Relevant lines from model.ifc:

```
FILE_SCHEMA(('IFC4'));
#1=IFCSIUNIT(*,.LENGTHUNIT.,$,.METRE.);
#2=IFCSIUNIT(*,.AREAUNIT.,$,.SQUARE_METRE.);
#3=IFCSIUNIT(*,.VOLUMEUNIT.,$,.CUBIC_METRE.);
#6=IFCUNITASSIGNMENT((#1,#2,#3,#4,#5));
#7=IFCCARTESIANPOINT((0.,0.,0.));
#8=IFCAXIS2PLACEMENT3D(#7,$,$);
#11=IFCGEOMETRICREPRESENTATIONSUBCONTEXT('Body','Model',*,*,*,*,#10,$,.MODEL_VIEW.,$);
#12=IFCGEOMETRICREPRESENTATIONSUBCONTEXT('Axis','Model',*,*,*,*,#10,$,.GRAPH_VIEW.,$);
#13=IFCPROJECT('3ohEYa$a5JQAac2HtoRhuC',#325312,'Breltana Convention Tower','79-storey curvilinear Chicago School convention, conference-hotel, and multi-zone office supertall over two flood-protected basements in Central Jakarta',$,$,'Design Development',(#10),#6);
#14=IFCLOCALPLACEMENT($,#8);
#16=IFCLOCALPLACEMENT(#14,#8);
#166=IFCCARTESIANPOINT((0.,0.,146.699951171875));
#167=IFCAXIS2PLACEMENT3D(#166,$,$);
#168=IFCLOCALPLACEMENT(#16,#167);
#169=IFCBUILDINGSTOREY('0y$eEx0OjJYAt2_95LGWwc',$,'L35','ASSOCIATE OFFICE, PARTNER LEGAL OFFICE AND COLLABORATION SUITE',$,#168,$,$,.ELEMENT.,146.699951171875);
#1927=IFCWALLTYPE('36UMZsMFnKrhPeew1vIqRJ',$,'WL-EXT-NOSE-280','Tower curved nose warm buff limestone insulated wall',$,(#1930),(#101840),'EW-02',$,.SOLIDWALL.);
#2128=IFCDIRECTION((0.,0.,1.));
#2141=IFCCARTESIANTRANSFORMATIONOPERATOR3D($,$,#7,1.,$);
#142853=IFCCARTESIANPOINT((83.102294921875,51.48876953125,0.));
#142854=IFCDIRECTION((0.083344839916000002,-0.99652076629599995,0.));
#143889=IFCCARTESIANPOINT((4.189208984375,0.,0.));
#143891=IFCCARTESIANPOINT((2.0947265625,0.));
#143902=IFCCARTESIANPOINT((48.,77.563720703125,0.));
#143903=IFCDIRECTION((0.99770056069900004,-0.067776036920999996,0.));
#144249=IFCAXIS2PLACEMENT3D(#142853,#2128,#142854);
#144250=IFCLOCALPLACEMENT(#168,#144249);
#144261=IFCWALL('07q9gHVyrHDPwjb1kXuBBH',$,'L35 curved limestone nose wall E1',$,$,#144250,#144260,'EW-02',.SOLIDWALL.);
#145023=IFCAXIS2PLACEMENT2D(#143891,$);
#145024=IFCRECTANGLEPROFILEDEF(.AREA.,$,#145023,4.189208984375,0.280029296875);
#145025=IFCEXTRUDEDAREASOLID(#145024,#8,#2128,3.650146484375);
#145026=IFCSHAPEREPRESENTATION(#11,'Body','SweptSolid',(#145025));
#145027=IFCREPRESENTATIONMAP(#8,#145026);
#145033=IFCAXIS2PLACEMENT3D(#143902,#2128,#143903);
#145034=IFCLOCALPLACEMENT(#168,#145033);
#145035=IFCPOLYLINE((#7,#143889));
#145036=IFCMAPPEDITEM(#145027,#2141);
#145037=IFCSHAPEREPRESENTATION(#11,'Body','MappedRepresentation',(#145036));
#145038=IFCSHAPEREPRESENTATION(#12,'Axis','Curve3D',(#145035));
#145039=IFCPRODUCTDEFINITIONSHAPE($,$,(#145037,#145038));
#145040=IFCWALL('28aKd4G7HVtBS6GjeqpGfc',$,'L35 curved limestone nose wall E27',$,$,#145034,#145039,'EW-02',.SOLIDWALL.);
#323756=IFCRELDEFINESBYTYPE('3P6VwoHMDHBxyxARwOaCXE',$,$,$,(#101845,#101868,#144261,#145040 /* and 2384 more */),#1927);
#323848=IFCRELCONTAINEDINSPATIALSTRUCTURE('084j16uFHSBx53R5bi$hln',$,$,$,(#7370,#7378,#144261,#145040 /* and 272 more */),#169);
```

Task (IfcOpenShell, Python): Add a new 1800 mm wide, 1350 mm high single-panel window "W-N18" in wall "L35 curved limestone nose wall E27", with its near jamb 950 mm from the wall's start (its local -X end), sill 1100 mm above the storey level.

```python
import numpy as np
import ifcopenshell
import ifcopenshell.api.feature
import ifcopenshell.api.geometry
import ifcopenshell.api.root
import ifcopenshell.api.spatial
import ifcopenshell.geom
import ifcopenshell.util.element
import ifcopenshell.util.placement
import ifcopenshell.util.representation
import ifcopenshell.util.shape
import ifcopenshell.util.unit

model = ifcopenshell.open("model.ifc")
unit_scale = ifcopenshell.util.unit.calculate_unit_scale(model)
settings = ifcopenshell.geom.settings()


def volume(element):
    """Net volume in cubic metres, openings subtracted."""
    shape = ifcopenshell.geom.create_shape(settings, element)
    return ifcopenshell.util.shape.get_volume(shape.geometry)


wall = model.by_id(145040)
storey = ifcopenshell.util.element.get_container(wall, ifc_class="IfcBuildingStorey")
context = ifcopenshell.util.representation.get_context(model, "Model", "Body", "MODEL_VIEW")
before = volume(wall)

width, height, from_end, sill = 1.8, 1.35, 0.95, 1.1  # metres

# The wall runs along its own X axis, and the end named is its -X end.
wall_shape = ifcopenshell.geom.create_shape(settings, wall)
x, y, z = ifcopenshell.util.shape.get_vertices(wall_shape.geometry).T
start = x.min() + from_end
face, thickness = float(y.min()), float(y.max() - y.min())
wall_matrix = ifcopenshell.util.placement.get_local_placement(wall.ObjectPlacement)
level = ifcopenshell.util.placement.get_local_placement(storey.ObjectPlacement)[2, 3]


def in_wall(x, y):
    """Placement at x, y metres in the wall's axes, at sill height."""
    matrix = wall_matrix.copy()
    matrix[:, 3] = wall_matrix @ np.array([x / unit_scale, y / unit_scale, 0.0, 1.0])
    matrix[2, 3] = level + sill / unit_scale
    return matrix


# Opening: a box that overshoots both wall faces by 50 mm.
opening = ifcopenshell.api.root.create_entity(model, ifc_class="IfcOpeningElement", predefined_type="OPENING")
box = ifcopenshell.api.geometry.add_wall_representation(
    model, context=context, length=width, height=height, thickness=thickness + 0.1
)
ifcopenshell.api.geometry.assign_representation(model, product=opening, representation=box)
ifcopenshell.api.geometry.edit_object_placement(model, product=opening, matrix=in_wall(start, face - 0.05), is_si=False)
ifcopenshell.api.feature.add_feature(model, feature=opening, element=wall)

window = ifcopenshell.api.root.create_entity(model, ifc_class="IfcWindow", name="W-N18", predefined_type="WINDOW")
window.OverallWidth, window.OverallHeight = width / unit_scale, height / unit_scale
window.PartitioningType = "SINGLE_PANEL"
body = ifcopenshell.api.geometry.add_window_representation(
    model,
    context=context,
    overall_width=window.OverallWidth,
    overall_height=window.OverallHeight,
    partition_type="SINGLE_PANEL",
)
ifcopenshell.api.geometry.assign_representation(model, product=window, representation=body)
ifcopenshell.api.spatial.assign_container(model, products=[window], relating_structure=storey)
ifcopenshell.api.feature.add_filling(model, opening=opening, element=window)

# Centre the window in the wall's thickness.
ifcopenshell.api.geometry.edit_object_placement(model, product=window, matrix=in_wall(start, face), is_si=False)
window_shape = ifcopenshell.geom.create_shape(settings, window)
depth = ifcopenshell.util.shape.get_vertices(window_shape.geometry)[:, 1]
offset = face + thickness / 2 - (depth.min() + depth.max()) / 2
ifcopenshell.api.geometry.edit_object_placement(model, product=window, matrix=in_wall(start, offset), is_si=False)

after = volume(wall)

print(f"wall volume {before:.3f} -> {after:.3f} m3")

model.write("model-out.ifc")
```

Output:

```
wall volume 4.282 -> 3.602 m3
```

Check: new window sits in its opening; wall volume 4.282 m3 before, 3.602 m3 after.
